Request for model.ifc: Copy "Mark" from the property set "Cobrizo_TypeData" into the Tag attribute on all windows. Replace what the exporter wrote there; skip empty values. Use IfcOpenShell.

First a look at what the model holds.

```python
import ifcopenshell
import ifcopenshell.util.element

model = ifcopenshell.open("model.ifc")
print(model.schema)
windows = model.by_type("IfcWindow")
print(len(windows), "windows")
for e in windows[:8]:
    source = ifcopenshell.util.element.get_pset(e, "Cobrizo_TypeData", "Mark")
    target = e.Tag
    print(e.id(), repr(source), repr(target), sep=" | ")
```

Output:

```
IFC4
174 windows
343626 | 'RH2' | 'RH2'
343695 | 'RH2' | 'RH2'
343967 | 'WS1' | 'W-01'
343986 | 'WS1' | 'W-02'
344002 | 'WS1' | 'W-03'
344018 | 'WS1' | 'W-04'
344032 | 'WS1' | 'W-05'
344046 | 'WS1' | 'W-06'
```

```python
import ifcopenshell
import ifcopenshell.util.element

model = ifcopenshell.open("model.ifc")

count = 0
for e in model.by_type("IfcWindow"):
    value = ifcopenshell.util.element.get_pset(e, "Cobrizo_TypeData", "Mark")
    current = e.Tag
    if not value or not value.strip() or current == value:
        continue
    e.Tag = value
    count += 1

print(count, "windows updated")

model.write("model-out.ifc")
```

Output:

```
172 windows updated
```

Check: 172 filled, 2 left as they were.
